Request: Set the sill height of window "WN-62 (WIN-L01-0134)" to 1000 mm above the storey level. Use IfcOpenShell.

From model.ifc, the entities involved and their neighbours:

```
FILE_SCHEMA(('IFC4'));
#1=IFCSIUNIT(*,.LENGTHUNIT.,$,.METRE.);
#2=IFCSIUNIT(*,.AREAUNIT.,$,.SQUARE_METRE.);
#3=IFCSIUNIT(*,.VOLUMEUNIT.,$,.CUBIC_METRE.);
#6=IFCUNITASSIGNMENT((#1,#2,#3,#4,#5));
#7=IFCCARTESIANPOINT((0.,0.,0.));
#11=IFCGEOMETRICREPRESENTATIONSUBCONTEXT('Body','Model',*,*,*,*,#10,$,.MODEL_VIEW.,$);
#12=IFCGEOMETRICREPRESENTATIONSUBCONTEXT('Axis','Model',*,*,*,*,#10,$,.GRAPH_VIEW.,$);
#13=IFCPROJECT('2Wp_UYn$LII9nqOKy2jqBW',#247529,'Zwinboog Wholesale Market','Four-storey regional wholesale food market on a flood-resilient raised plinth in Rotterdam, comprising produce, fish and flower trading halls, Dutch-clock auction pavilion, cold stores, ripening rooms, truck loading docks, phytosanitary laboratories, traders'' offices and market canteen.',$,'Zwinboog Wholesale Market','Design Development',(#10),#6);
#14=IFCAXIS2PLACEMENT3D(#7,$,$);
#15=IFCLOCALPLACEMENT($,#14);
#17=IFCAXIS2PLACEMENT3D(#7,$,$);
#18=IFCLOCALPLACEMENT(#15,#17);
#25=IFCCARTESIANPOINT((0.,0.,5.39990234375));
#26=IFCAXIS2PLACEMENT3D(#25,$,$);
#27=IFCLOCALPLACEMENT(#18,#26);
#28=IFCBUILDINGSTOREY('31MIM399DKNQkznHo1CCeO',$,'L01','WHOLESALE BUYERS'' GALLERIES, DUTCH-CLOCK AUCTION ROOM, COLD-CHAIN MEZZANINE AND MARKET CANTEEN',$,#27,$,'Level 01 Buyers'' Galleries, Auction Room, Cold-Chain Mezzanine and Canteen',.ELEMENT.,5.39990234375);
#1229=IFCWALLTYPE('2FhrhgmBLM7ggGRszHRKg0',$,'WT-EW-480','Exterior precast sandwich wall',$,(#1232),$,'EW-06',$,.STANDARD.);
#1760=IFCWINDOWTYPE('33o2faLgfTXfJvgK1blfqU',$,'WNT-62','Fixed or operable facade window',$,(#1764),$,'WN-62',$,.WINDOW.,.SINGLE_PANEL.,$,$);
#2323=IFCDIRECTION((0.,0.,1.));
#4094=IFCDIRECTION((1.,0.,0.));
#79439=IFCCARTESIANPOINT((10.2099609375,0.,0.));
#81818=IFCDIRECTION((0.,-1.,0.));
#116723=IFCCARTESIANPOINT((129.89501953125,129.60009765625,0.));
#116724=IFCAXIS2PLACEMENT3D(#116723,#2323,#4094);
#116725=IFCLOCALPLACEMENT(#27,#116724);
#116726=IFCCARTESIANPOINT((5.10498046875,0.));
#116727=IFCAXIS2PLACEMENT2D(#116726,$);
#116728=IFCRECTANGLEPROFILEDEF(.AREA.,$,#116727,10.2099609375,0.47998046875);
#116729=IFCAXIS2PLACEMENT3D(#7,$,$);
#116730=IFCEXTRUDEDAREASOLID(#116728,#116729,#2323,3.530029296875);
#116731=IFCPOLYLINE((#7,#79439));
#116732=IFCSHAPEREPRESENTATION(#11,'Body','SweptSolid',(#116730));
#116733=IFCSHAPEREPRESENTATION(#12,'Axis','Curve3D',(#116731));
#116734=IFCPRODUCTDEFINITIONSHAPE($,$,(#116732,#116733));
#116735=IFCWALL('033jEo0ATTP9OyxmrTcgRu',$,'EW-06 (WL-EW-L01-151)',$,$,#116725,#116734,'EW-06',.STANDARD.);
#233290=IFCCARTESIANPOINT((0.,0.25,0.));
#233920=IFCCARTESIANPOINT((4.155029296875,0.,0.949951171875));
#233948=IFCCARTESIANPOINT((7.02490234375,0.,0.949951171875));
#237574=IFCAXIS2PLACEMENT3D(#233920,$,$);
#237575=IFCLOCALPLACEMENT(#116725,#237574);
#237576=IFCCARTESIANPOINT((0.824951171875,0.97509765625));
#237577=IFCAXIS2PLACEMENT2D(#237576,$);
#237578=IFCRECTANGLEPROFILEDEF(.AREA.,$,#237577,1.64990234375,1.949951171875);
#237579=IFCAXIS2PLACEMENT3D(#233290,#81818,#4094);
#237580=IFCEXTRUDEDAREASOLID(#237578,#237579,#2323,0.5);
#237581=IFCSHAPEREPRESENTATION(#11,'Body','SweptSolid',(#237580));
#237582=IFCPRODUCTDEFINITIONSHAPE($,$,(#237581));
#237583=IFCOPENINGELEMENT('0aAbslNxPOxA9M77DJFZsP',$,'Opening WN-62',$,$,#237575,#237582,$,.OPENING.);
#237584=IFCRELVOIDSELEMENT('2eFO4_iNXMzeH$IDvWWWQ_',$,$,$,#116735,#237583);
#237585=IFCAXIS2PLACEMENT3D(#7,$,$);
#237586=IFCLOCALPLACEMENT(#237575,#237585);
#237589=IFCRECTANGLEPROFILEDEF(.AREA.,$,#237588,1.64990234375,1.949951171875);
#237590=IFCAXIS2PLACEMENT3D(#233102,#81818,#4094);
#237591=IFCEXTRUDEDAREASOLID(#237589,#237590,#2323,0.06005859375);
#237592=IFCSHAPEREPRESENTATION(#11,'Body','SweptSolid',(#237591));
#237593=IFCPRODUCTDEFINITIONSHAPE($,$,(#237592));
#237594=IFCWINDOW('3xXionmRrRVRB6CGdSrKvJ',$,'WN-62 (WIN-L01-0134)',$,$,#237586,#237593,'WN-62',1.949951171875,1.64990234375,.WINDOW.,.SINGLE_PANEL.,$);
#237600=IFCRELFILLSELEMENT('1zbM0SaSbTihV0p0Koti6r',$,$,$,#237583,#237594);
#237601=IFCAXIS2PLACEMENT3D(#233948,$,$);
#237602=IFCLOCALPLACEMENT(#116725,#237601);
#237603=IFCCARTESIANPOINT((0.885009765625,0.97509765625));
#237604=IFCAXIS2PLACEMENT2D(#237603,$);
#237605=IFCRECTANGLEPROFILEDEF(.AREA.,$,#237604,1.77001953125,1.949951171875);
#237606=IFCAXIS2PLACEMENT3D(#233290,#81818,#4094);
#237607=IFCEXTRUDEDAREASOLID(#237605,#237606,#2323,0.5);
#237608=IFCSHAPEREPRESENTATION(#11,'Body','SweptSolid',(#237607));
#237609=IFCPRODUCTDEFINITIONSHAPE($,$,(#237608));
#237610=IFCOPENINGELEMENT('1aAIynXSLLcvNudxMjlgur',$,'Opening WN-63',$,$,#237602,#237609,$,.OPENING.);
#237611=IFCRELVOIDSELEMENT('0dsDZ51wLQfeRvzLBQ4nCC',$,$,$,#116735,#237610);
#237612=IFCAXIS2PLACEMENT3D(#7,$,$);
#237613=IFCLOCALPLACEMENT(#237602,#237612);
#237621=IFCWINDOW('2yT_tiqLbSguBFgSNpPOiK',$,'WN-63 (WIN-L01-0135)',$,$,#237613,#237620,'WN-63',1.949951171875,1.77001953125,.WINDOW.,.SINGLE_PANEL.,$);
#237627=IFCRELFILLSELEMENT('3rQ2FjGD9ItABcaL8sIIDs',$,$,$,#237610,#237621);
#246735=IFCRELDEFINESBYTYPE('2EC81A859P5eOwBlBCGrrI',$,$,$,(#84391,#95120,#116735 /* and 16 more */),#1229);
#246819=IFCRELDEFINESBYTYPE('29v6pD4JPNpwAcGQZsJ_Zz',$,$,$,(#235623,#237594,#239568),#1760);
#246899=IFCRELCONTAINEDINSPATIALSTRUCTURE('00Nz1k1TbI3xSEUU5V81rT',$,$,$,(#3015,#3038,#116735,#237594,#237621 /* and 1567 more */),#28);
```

```python
import numpy as np
import ifcopenshell
import ifcopenshell.api.geometry
import ifcopenshell.geom
import ifcopenshell.util.element
import ifcopenshell.util.placement
import ifcopenshell.util.shape
import ifcopenshell.util.unit

model = ifcopenshell.open("model.ifc")
unit_scale = ifcopenshell.util.unit.calculate_unit_scale(model)

window = model.by_guid("3xXionmRrRVRB6CGdSrKvJ")
opening = window.FillsVoids[0].RelatingOpeningElement
storey = ifcopenshell.util.element.get_container(window, ifc_class="IfcBuildingStorey")
level = ifcopenshell.util.placement.get_local_placement(storey.ObjectPlacement)[2, 3]

# The opening's origin need not be at the sill, so measure its lowest point.
shape = ifcopenshell.geom.create_shape(ifcopenshell.geom.settings(), opening)
bottom = ifcopenshell.util.shape.get_shape_bottom_elevation(shape, shape.geometry) / unit_scale
dz = level + 1 / unit_scale - bottom

shift = np.array([0.0, 0.0, dz])
# The window is placed relative to its opening, so it follows when the opening moves.
matrix = ifcopenshell.util.placement.get_local_placement(opening.ObjectPlacement)
matrix[:3, 3] += shift
ifcopenshell.api.geometry.edit_object_placement(
    model, product=opening, matrix=matrix, is_si=False, should_transform_children=True
)

print(f"moved by {dz * unit_scale:+.3f} m")

model.write("model_v2.ifc")
```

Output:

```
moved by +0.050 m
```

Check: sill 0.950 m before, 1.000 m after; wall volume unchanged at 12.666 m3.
